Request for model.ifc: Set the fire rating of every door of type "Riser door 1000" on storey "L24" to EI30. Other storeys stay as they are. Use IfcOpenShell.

First a look at what the model holds.

```python
import ifcopenshell
import ifcopenshell.util.element

model = ifcopenshell.open("model.ifc")
print(model.schema)
storey = next(s for s in model.by_type("IfcBuildingStorey") if s.Name == "L24")
doors = [e for e in ifcopenshell.util.element.get_decomposition(storey) if e.is_a("IfcDoor")]
seen = {}
for e in doors:
    element_type = ifcopenshell.util.element.get_type(e)
    key = (element_type.Name if element_type != e and element_type else None, ifcopenshell.util.element.get_pset(e, "Pset_DoorCommon", "FireRating"))
    seen[key] = seen.get(key, 0) + 1
for (name, value), count in sorted(seen.items(), key=str):
    print(count, "x", name, "|", value)
```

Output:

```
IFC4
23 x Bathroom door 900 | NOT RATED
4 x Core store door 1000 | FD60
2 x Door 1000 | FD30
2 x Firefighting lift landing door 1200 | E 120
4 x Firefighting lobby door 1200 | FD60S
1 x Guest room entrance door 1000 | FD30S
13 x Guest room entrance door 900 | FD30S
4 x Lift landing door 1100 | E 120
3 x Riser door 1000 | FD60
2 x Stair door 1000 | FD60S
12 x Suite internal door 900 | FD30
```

```python
import ifcopenshell
import ifcopenshell.api.pset
import ifcopenshell.util.element

model = ifcopenshell.open("model.ifc")

storey = next(s for s in model.by_type("IfcBuildingStorey") if s.Name == "L24")
doors = [e for e in ifcopenshell.util.element.get_decomposition(storey) if e.is_a("IfcDoor")]

count = 0
for e in doors:
    element_type = ifcopenshell.util.element.get_type(e)
    if element_type in (None, e) or element_type.Name != "Riser door 1000":
        continue
    # add_pset returns the element's existing set when there is one.
    pset = ifcopenshell.api.pset.add_pset(model, product=e, name="Pset_DoorCommon")
    ifcopenshell.api.pset.edit_pset(model, pset=pset, properties={"FireRating": "EI30"})
    count += 1

print(count, "doors updated")

model.write("model-out.ifc")
```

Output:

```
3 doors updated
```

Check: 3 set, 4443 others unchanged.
